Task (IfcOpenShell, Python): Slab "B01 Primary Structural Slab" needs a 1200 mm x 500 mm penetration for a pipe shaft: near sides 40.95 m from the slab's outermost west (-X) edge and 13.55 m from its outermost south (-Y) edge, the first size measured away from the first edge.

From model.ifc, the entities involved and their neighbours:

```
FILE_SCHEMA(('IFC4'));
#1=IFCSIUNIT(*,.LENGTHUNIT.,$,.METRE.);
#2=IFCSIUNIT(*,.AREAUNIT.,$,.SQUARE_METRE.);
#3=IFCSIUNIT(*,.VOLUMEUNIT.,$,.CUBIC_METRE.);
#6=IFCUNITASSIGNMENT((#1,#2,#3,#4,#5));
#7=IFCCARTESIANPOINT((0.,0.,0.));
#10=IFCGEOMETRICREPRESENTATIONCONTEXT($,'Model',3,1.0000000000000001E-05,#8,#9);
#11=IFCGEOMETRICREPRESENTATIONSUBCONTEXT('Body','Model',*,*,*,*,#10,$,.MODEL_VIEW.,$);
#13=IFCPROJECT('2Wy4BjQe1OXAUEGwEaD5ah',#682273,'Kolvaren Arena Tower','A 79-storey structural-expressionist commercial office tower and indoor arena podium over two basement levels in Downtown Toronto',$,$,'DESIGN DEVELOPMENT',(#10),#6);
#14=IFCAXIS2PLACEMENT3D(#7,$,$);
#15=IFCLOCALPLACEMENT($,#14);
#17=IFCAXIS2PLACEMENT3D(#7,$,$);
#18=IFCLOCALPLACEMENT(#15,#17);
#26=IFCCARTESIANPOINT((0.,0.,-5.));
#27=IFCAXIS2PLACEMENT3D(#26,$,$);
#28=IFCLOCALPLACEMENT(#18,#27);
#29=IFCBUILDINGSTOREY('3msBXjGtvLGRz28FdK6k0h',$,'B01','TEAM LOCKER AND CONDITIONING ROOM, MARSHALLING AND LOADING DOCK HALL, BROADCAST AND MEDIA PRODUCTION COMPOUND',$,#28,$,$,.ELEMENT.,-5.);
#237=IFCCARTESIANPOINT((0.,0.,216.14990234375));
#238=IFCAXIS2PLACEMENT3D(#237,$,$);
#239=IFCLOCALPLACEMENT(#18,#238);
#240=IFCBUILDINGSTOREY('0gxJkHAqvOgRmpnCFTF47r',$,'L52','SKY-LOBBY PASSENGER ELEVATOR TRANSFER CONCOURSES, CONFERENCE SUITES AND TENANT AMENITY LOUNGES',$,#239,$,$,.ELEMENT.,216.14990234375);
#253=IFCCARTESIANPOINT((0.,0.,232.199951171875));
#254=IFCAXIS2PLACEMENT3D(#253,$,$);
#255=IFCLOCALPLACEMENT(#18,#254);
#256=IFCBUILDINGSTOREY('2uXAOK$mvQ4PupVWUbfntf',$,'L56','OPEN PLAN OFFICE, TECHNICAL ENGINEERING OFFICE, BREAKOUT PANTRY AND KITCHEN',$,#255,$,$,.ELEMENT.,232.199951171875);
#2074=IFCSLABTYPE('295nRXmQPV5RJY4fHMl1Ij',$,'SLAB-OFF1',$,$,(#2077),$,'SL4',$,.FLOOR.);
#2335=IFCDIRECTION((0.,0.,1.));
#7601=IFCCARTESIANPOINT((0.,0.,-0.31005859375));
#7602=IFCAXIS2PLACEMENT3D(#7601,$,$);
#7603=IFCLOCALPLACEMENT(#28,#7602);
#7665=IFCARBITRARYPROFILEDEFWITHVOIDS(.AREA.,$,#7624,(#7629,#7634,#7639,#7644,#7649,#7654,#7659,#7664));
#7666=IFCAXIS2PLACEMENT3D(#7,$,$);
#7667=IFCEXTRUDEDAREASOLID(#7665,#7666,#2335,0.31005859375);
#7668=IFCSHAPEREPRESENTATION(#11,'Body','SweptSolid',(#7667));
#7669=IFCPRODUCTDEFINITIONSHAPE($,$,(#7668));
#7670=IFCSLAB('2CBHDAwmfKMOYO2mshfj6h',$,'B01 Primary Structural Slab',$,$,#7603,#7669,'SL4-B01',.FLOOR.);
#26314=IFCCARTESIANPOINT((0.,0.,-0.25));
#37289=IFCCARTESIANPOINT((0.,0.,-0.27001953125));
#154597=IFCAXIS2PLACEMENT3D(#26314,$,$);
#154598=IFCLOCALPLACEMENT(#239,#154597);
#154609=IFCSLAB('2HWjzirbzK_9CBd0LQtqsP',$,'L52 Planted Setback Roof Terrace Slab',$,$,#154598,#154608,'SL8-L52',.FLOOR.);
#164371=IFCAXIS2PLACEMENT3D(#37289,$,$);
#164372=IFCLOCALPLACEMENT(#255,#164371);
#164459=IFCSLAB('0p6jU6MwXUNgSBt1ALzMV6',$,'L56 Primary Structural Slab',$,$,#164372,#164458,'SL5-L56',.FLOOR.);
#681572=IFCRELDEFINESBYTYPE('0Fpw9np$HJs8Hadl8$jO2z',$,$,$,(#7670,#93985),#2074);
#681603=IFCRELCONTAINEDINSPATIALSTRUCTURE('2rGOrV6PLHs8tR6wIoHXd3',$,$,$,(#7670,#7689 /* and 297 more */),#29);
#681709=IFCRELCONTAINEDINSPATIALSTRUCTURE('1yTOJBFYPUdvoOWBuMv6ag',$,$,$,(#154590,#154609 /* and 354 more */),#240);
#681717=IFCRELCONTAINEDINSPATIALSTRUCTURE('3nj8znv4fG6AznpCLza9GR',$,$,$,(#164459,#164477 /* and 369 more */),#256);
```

```python
import numpy as np
import ifcopenshell
import ifcopenshell.api.feature
import ifcopenshell.api.geometry
import ifcopenshell.api.root
import ifcopenshell.geom
import ifcopenshell.util.placement
import ifcopenshell.util.representation
import ifcopenshell.util.shape
import ifcopenshell.util.unit

model = ifcopenshell.open("model.ifc")
unit_scale = ifcopenshell.util.unit.calculate_unit_scale(model)
settings = ifcopenshell.geom.settings()


def volume(element):
    """Net volume in cubic metres, openings subtracted."""
    shape = ifcopenshell.geom.create_shape(settings, element)
    return ifcopenshell.util.shape.get_volume(shape.geometry)


slab = model.by_id(7670)
before = volume(slab)

# Extent in the slab's own axes, in metres. The edges named are its -X and -Y sides.
slab_shape = ifcopenshell.geom.create_shape(settings, slab)
vertices = ifcopenshell.util.shape.get_vertices(slab_shape.geometry)
x_min, y_min, bottom = vertices.min(axis=0)
top = vertices[:, 2].max()

opening = ifcopenshell.api.root.create_entity(model, ifc_class="IfcOpeningElement", name="Pipe shaft opening", predefined_type="OPENING")
context = ifcopenshell.util.representation.get_context(model, "Model", "Body", "MODEL_VIEW")
width, depth = 1.2, 0.5
outline = [(0.0, 0.0), (width, 0.0), (width, depth), (0.0, depth), (0.0, 0.0)]
# Overshoot both faces by 50 mm so the cut is clean.
shape = ifcopenshell.api.geometry.add_slab_representation(
    model, context=context, depth=top - bottom + 0.1, polyline=outline
)
ifcopenshell.api.geometry.assign_representation(model, product=opening, representation=shape)

matrix = ifcopenshell.util.placement.get_local_placement(slab.ObjectPlacement)
matrix[:, 3] = matrix @ np.append(np.array([x_min + 40.95, y_min + 13.55, bottom - 0.05]) / unit_scale, 1.0)
ifcopenshell.api.geometry.edit_object_placement(model, product=opening, matrix=matrix, is_si=False)
ifcopenshell.api.feature.add_feature(model, feature=opening, element=slab)

after = volume(slab)

print(f"slab volume {before:.3f} -> {after:.3f} m3")

model.write("model_v2.ifc")
```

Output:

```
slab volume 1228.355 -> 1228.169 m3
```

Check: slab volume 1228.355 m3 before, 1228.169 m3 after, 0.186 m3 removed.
